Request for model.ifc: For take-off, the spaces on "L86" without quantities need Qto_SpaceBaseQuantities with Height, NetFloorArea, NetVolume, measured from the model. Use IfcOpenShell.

First a look at what the model holds.

```python
import ifcopenshell
import ifcopenshell.util.element
import ifcopenshell.util.unit

model = ifcopenshell.open("model.ifc")
print(model.schema)
for unit_type in ("LENGTHUNIT", "AREAUNIT", "VOLUMEUNIT"):
    print(unit_type, ifcopenshell.util.unit.calculate_unit_scale(model, unit_type))
storey = next(s for s in model.by_type("IfcBuildingStorey") if s.Name == "L86")
spaces = [e for e in ifcopenshell.util.element.get_decomposition(storey) if e.is_a("IfcSpace")]
for e in sorted(spaces, key=lambda e: e.id()):
    print(e.id(), e.is_a(), e.Name, list(ifcopenshell.util.element.get_psets(e, qtos_only=True)), sep=" | ")
```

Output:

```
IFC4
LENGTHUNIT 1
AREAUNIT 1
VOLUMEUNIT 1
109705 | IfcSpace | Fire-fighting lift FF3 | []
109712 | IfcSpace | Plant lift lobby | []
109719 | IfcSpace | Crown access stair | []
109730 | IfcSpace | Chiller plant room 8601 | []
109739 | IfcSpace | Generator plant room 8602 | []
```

```python
import ifcopenshell
import ifcopenshell.api.pset
import ifcopenshell.geom
import ifcopenshell.util.element
import ifcopenshell.util.shape
import ifcopenshell.util.unit

model = ifcopenshell.open("model.ifc")
unit_scale = ifcopenshell.util.unit.calculate_unit_scale(model)
area_scale = ifcopenshell.util.unit.calculate_unit_scale(model, "AREAUNIT")
volume_scale = ifcopenshell.util.unit.calculate_unit_scale(model, "VOLUMEUNIT")
settings = ifcopenshell.geom.settings()

storey = next(s for s in model.by_type("IfcBuildingStorey") if s.Name == "L86")
spaces = [e for e in ifcopenshell.util.element.get_decomposition(storey) if e.is_a("IfcSpace")]

for e in sorted(spaces, key=lambda e: e.id()):
    if ifcopenshell.util.element.get_psets(e, qtos_only=True, should_inherit=False):
        continue
    # Geometry comes back in metres, in the element's own axes.
    shape = ifcopenshell.geom.create_shape(settings, e)
    values = {
        "Height": ifcopenshell.util.shape.get_z(shape.geometry) / unit_scale,
        "NetFloorArea": ifcopenshell.util.shape.get_footprint_area(shape.geometry) / area_scale,
        "NetVolume": ifcopenshell.util.shape.get_volume(shape.geometry) / volume_scale,
    }
    qto = ifcopenshell.api.pset.add_qto(model, product=e, name="Qto_SpaceBaseQuantities")
    ifcopenshell.api.pset.edit_qto(model, qto=qto, properties=values)
    print(e.id(), {k: round(v, 3) for k, v in values.items()})

model.write("model_rev.ifc")
```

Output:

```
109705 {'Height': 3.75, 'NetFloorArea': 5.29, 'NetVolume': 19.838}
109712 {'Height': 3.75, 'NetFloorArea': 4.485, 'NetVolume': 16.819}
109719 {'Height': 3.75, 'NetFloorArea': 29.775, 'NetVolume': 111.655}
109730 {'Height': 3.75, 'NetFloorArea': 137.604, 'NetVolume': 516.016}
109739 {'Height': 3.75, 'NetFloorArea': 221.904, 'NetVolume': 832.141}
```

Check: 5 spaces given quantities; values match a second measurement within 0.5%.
